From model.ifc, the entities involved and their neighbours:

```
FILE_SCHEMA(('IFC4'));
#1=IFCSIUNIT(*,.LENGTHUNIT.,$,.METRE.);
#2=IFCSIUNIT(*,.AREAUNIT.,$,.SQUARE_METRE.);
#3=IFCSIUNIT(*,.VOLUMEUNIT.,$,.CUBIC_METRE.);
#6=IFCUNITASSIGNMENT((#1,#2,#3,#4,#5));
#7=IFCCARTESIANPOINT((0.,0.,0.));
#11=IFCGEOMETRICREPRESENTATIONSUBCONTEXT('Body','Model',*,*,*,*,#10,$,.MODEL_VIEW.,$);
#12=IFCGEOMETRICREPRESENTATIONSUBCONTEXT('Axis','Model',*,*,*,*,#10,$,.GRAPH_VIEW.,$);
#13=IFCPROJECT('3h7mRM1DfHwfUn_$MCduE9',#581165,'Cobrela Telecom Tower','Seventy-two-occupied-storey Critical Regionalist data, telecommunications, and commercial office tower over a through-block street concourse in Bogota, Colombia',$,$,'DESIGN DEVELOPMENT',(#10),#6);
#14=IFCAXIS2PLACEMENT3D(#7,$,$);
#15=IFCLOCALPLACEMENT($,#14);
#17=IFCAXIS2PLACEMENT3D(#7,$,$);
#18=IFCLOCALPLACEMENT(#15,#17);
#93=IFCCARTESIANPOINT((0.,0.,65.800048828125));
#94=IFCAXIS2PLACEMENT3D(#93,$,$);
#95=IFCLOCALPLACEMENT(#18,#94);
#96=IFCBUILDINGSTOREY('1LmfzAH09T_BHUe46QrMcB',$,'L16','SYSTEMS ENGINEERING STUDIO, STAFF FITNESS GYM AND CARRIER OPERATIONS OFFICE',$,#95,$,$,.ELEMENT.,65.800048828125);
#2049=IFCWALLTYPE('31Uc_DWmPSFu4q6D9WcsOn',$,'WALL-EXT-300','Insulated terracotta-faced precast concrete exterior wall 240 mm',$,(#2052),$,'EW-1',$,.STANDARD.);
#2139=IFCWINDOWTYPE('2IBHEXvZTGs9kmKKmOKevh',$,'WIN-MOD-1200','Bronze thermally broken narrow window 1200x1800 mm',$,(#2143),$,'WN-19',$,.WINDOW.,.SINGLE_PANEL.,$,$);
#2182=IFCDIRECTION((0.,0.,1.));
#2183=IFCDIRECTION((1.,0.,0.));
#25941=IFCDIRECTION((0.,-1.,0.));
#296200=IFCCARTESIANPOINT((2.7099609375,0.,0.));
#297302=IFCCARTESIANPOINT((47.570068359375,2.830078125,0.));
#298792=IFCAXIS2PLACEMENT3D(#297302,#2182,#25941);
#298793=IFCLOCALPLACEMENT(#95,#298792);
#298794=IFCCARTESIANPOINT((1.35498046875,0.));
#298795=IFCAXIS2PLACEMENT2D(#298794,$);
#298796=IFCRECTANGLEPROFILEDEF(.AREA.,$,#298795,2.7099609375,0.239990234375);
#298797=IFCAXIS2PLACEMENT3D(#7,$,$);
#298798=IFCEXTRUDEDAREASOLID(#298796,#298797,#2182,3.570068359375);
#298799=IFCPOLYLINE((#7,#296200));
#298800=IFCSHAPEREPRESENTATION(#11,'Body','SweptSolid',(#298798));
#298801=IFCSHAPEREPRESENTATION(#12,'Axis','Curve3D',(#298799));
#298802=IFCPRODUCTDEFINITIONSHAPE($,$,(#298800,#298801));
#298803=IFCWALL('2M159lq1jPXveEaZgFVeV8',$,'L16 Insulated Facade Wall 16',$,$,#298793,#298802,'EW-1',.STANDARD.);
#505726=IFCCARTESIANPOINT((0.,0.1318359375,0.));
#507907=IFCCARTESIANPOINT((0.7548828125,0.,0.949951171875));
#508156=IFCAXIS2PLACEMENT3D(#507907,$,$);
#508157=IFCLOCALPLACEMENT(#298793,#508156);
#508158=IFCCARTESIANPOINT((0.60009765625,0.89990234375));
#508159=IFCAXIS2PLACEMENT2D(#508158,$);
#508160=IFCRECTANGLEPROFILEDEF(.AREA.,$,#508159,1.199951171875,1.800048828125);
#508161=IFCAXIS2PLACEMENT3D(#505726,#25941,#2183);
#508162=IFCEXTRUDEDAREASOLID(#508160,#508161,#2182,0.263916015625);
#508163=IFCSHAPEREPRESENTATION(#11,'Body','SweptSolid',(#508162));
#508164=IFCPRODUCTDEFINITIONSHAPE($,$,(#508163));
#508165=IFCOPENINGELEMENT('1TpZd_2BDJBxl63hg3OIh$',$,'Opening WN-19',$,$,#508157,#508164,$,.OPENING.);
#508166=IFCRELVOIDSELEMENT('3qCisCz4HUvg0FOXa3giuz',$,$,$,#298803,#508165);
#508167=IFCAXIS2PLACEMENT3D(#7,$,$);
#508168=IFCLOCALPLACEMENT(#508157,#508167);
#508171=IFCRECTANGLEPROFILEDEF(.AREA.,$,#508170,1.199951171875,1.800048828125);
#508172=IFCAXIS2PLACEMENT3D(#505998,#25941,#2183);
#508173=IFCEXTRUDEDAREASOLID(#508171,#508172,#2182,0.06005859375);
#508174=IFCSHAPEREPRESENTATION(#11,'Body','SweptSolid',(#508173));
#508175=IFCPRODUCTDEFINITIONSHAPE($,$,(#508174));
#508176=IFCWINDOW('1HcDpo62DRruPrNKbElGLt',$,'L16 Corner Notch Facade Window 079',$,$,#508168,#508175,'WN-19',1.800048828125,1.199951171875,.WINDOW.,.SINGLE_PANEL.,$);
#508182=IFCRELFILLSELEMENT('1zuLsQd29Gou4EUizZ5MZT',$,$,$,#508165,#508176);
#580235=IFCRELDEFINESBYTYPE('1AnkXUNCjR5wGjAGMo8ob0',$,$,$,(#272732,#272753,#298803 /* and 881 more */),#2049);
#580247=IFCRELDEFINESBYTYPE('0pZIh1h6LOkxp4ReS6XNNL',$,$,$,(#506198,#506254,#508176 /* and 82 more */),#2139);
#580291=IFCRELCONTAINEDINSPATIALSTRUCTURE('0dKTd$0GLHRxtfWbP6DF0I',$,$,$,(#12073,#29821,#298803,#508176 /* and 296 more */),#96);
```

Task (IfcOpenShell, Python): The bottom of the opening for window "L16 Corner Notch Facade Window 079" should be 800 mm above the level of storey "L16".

```python
import numpy as np
import ifcopenshell
import ifcopenshell.api.geometry
import ifcopenshell.geom
import ifcopenshell.util.element
import ifcopenshell.util.placement
import ifcopenshell.util.shape
import ifcopenshell.util.unit

model = ifcopenshell.open("model.ifc")
unit_scale = ifcopenshell.util.unit.calculate_unit_scale(model)

window = model.by_guid("1HcDpo62DRruPrNKbElGLt")
opening = window.FillsVoids[0].RelatingOpeningElement
storey = ifcopenshell.util.element.get_container(window, ifc_class="IfcBuildingStorey")
level = ifcopenshell.util.placement.get_local_placement(storey.ObjectPlacement)[2, 3]

# The opening's origin need not be at the sill, so measure its lowest point.
shape = ifcopenshell.geom.create_shape(ifcopenshell.geom.settings(), opening)
bottom = ifcopenshell.util.shape.get_shape_bottom_elevation(shape, shape.geometry) / unit_scale
dz = level + 0.8 - bottom

shift = np.array([0.0, 0.0, dz])
# The window is placed relative to its opening, so it follows when the opening moves.
matrix = ifcopenshell.util.placement.get_local_placement(opening.ObjectPlacement)
matrix[:3, 3] += shift
ifcopenshell.api.geometry.edit_object_placement(
    model, product=opening, matrix=matrix, is_si=False, should_transform_children=True
)

print(f"moved by {dz * unit_scale:+.3f} m")

model.write("model_edited.ifc")
```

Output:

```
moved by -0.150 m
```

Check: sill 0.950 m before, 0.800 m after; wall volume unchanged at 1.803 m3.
